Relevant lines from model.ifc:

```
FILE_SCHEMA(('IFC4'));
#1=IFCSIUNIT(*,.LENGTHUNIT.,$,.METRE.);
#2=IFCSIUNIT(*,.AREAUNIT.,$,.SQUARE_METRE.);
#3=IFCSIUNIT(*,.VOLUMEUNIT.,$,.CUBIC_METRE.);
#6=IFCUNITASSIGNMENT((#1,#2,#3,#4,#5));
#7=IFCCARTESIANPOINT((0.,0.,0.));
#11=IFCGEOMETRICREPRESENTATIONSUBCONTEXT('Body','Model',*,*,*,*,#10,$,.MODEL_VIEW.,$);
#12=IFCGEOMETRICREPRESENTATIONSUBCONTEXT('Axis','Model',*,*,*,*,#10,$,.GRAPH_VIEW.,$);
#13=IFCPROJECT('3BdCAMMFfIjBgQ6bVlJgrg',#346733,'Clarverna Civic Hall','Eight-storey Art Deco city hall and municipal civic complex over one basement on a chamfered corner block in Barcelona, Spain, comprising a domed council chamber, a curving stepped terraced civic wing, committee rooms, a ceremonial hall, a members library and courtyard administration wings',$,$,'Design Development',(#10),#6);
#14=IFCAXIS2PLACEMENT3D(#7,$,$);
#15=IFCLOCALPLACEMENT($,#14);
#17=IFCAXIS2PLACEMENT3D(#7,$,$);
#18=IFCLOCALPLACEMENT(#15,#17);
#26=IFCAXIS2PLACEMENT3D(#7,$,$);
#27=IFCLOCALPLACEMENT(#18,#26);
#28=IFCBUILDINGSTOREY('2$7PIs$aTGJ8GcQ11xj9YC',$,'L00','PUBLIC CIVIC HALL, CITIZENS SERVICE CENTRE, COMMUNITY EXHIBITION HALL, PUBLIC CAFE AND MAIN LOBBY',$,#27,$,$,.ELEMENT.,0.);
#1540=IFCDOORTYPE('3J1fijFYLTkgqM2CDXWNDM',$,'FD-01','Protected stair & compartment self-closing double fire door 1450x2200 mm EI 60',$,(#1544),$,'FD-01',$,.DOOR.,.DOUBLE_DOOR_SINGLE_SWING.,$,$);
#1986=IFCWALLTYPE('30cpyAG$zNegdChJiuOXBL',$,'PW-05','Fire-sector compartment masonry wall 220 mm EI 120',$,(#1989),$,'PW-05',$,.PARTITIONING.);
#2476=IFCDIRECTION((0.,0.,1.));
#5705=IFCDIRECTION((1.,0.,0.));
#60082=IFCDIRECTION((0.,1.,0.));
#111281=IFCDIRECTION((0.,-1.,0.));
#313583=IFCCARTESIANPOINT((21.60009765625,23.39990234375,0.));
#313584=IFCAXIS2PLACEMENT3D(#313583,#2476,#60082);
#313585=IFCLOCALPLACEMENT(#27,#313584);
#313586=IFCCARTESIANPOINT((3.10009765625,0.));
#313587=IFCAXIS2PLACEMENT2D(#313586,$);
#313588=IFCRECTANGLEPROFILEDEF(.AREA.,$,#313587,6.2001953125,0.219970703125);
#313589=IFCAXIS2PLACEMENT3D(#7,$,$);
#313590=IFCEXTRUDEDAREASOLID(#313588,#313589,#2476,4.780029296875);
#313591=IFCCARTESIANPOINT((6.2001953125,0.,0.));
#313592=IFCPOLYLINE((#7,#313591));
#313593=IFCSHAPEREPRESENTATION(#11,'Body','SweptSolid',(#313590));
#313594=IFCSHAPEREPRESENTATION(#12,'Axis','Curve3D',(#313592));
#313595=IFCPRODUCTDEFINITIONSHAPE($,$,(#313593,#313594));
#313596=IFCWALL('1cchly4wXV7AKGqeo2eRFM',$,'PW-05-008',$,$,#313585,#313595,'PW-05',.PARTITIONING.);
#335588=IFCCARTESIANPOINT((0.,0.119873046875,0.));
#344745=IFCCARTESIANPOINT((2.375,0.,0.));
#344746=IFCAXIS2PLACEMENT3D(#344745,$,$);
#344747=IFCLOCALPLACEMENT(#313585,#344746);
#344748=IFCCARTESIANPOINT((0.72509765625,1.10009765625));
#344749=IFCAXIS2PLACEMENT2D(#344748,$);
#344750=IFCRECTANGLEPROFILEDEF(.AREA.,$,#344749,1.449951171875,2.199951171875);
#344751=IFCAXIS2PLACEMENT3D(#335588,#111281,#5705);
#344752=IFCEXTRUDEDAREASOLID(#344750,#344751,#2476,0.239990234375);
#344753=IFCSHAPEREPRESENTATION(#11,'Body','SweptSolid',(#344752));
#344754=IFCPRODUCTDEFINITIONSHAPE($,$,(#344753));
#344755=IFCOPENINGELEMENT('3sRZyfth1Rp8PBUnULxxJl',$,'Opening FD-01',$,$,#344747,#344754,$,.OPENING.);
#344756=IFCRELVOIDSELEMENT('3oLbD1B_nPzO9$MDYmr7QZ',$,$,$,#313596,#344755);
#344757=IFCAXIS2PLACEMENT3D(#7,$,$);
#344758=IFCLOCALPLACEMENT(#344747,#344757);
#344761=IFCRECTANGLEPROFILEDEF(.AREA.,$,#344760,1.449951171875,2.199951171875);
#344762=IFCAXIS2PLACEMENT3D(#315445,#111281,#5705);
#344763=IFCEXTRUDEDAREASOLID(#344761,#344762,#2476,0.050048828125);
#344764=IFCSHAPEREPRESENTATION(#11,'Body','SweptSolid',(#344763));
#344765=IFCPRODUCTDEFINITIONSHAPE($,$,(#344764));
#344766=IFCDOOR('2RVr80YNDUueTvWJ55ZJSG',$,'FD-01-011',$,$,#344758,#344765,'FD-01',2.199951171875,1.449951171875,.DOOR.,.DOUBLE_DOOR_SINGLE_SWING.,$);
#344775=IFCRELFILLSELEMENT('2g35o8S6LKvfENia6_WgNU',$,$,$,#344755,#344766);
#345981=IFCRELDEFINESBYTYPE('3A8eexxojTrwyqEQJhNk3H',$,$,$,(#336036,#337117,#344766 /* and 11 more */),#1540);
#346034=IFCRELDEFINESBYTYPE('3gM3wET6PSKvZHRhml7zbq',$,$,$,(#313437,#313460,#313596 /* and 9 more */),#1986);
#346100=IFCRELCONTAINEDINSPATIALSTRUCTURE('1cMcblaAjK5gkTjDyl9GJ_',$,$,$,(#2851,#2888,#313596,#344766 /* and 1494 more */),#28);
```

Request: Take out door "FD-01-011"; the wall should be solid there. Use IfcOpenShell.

```python
import ifcopenshell
import ifcopenshell.api.feature
import ifcopenshell.api.root
import ifcopenshell.geom
import ifcopenshell.util.shape

model = ifcopenshell.open("model.ifc")
settings = ifcopenshell.geom.settings()


def volume(element):
    """Net volume in cubic metres, openings subtracted."""
    shape = ifcopenshell.geom.create_shape(settings, element)
    return ifcopenshell.util.shape.get_volume(shape.geometry)


door = model.by_guid("2RVr80YNDUueTvWJ55ZJSG")
opening = door.FillsVoids[0].RelatingOpeningElement
wall = opening.VoidsElements[0].RelatingBuildingElement
before = volume(wall)

ifcopenshell.api.root.remove_product(model, product=door)
ifcopenshell.api.feature.remove_feature(model, feature=opening)

after = volume(wall)

print(f"wall volume {before:.3f} -> {after:.3f} m3")

model.write("model_updated.ifc")
```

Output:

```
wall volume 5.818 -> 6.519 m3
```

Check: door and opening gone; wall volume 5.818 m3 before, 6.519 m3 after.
